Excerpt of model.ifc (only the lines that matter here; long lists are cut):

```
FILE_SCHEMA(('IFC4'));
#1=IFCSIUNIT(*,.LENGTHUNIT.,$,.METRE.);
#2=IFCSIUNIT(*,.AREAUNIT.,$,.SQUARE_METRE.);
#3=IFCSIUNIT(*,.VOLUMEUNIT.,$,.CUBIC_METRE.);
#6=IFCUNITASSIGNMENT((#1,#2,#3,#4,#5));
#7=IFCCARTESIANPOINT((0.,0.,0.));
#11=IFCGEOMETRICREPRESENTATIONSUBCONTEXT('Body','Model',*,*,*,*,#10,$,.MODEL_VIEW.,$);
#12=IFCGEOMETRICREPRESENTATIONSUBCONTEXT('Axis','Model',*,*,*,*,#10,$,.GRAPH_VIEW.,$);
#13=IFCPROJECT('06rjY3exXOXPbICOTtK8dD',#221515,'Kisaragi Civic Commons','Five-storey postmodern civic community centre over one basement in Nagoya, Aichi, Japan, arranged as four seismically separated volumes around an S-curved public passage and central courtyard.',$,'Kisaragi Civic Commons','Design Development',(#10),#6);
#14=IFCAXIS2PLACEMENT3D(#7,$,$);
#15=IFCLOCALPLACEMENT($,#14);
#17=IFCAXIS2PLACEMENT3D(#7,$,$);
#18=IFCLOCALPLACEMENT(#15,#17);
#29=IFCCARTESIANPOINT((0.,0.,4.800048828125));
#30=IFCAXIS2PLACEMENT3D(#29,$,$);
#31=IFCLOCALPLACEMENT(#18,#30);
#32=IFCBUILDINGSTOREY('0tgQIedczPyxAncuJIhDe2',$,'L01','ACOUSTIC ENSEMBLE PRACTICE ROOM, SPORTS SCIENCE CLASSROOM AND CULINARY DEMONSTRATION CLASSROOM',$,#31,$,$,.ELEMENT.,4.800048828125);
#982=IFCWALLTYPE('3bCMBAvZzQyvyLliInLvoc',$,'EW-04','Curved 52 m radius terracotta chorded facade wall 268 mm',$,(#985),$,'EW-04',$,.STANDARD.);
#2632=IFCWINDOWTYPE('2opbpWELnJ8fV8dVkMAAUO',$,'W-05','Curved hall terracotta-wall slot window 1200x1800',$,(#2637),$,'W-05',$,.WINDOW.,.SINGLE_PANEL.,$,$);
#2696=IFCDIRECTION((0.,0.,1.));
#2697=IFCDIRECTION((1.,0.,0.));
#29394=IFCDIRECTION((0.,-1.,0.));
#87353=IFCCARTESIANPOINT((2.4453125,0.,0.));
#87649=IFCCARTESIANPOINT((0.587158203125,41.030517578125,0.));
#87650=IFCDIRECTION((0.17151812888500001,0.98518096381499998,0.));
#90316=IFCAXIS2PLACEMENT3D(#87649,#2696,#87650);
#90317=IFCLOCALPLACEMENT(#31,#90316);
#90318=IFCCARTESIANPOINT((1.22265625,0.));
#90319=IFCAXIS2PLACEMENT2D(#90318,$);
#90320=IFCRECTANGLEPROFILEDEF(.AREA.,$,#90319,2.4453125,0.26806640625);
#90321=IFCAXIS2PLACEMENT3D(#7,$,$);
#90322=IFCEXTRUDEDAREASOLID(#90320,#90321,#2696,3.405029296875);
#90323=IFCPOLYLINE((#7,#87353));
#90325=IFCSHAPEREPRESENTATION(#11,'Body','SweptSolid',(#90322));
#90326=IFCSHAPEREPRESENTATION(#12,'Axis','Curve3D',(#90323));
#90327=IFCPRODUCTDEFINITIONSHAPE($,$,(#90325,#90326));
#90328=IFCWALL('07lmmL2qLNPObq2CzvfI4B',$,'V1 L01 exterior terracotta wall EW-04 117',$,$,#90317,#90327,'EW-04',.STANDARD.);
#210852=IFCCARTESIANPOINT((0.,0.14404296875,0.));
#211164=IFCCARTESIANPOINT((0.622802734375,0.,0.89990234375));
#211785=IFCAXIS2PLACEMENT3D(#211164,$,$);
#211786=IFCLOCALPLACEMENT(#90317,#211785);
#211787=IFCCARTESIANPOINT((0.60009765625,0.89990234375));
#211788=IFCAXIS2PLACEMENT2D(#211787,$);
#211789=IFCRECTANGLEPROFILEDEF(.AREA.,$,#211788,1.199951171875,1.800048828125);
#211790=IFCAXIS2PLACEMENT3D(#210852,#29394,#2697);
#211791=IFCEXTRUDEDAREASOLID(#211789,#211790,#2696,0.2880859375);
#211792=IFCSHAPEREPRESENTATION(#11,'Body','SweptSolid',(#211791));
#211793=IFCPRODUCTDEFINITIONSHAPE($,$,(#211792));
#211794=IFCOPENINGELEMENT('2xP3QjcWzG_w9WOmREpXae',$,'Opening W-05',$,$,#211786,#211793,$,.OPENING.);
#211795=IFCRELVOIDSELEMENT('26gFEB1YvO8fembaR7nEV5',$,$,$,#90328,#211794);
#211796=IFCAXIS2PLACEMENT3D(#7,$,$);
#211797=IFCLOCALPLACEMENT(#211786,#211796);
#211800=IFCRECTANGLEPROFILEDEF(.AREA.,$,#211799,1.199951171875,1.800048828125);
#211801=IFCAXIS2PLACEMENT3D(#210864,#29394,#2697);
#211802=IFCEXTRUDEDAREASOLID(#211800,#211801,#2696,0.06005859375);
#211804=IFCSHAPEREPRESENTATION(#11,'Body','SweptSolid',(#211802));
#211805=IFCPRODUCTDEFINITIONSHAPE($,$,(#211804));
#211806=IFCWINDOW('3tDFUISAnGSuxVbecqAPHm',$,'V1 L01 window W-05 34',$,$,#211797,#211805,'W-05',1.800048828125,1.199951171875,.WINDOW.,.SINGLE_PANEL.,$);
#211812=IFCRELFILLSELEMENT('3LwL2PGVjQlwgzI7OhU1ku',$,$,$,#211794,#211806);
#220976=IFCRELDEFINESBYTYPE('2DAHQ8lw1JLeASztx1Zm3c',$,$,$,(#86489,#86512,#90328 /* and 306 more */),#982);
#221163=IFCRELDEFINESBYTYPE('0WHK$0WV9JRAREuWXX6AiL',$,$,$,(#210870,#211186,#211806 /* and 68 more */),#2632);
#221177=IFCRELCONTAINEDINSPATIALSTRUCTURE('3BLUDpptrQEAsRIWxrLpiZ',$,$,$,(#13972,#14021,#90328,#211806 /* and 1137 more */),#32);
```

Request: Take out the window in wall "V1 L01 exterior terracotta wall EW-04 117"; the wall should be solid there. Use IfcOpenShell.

```python
import ifcopenshell
import ifcopenshell.api.feature
import ifcopenshell.api.root
import ifcopenshell.geom
import ifcopenshell.util.shape

model = ifcopenshell.open("model.ifc")
settings = ifcopenshell.geom.settings()


def volume(element):
    """Net volume in cubic metres, openings subtracted."""
    shape = ifcopenshell.geom.create_shape(settings, element)
    return ifcopenshell.util.shape.get_volume(shape.geometry)


window = model.by_id(211806)
opening = window.FillsVoids[0].RelatingOpeningElement
wall = opening.VoidsElements[0].RelatingBuildingElement
before = volume(wall)

ifcopenshell.api.root.remove_product(model, product=window)
ifcopenshell.api.feature.remove_feature(model, feature=opening)

after = volume(wall)

print(f"wall volume {before:.3f} -> {after:.3f} m3")

model.write("model_edited.ifc")
```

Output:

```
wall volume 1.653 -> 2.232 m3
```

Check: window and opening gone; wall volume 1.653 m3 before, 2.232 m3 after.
